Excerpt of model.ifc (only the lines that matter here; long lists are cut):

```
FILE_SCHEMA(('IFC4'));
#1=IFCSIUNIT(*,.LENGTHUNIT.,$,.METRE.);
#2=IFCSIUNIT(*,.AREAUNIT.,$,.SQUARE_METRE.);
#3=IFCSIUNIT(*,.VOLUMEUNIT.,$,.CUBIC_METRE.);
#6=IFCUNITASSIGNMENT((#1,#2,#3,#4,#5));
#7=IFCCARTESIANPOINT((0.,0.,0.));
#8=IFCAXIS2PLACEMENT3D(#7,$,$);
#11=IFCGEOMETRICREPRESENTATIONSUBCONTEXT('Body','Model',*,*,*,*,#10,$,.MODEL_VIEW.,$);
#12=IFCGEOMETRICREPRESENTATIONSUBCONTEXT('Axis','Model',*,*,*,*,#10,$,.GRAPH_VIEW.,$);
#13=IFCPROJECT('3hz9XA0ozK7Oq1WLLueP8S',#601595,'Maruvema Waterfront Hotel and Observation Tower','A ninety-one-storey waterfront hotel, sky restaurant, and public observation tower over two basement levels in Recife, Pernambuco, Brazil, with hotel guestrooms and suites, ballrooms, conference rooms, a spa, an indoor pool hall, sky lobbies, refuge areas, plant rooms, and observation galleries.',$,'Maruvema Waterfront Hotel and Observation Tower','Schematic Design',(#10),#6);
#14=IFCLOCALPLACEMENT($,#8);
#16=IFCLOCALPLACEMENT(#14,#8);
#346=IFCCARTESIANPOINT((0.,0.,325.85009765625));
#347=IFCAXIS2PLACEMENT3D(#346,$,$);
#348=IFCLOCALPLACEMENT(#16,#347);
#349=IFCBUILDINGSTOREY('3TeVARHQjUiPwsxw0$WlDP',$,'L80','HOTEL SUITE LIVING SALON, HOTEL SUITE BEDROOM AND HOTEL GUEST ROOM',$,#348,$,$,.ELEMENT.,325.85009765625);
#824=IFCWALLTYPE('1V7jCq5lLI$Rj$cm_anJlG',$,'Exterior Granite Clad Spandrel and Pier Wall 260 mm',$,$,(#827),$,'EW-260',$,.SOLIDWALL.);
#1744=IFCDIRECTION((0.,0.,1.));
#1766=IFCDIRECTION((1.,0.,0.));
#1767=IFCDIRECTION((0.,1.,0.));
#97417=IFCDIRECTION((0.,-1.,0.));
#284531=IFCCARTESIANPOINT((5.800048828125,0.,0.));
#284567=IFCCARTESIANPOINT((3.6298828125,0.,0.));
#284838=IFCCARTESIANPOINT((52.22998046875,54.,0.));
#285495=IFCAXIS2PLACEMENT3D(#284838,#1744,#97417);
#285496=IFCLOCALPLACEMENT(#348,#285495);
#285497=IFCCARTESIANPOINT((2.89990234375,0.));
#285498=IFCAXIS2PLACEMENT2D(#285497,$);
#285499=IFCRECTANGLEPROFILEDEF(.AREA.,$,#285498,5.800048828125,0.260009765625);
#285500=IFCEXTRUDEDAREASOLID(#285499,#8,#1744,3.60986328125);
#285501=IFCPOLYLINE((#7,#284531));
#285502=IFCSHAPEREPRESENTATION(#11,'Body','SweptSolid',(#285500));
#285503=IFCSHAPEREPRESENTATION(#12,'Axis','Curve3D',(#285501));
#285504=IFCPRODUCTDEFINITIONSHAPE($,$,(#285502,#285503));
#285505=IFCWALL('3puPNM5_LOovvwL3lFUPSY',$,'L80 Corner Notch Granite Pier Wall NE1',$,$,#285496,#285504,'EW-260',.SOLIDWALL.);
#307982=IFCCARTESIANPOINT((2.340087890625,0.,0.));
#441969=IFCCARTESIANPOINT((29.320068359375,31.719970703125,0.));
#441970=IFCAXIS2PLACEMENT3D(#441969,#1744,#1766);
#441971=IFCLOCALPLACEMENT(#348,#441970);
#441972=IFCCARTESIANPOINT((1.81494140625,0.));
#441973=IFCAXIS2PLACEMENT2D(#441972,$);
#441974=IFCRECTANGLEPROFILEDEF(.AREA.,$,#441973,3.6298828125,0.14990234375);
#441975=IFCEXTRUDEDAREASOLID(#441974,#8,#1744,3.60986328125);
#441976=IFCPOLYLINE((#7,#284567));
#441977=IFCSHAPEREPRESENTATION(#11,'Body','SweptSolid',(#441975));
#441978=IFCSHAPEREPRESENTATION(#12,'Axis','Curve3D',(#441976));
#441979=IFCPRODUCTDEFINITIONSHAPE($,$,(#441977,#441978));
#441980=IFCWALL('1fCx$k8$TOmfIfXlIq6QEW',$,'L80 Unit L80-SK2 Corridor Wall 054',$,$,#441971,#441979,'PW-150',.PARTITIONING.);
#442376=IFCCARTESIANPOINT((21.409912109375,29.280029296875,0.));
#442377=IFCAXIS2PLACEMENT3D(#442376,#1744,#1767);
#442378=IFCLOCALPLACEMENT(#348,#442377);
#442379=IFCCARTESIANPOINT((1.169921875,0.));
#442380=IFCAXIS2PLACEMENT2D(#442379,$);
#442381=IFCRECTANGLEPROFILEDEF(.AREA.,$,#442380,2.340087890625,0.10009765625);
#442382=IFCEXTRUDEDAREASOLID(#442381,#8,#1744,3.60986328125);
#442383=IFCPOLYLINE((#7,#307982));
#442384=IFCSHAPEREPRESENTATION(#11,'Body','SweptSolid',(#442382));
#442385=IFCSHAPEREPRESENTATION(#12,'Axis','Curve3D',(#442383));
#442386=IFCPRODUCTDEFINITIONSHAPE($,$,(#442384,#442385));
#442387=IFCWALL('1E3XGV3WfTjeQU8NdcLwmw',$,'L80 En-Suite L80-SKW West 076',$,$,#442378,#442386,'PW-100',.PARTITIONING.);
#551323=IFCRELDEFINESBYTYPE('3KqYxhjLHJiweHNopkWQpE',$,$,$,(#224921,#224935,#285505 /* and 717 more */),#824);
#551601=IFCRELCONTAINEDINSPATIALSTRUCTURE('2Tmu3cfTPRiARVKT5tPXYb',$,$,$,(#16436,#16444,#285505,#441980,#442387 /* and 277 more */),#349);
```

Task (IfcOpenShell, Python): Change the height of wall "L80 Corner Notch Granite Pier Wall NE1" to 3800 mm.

```python
import ifcopenshell
import ifcopenshell.geom
import ifcopenshell.util.representation
import ifcopenshell.util.shape
import ifcopenshell.util.unit

model = ifcopenshell.open("model.ifc")
unit_scale = ifcopenshell.util.unit.calculate_unit_scale(model)
settings = ifcopenshell.geom.settings()


def volume(element):
    """Net volume in cubic metres, openings subtracted."""
    shape = ifcopenshell.geom.create_shape(settings, element)
    return ifcopenshell.util.shape.get_volume(shape.geometry)


wall = model.by_id(285505)
before = volume(wall)

body = ifcopenshell.util.representation.get_representation(wall, "Model", "Body")
solid = body.Items[0]
old_height = solid.Depth
solid.Depth = 3.8 / unit_scale
after = volume(wall)

print(f"height {old_height:g} -> {solid.Depth:g}, volume {before:.3f} -> {after:.3f} m3")

model.write("model_v2.ifc")
```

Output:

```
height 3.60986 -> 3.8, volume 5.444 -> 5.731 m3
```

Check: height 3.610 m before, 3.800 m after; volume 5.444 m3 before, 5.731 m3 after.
